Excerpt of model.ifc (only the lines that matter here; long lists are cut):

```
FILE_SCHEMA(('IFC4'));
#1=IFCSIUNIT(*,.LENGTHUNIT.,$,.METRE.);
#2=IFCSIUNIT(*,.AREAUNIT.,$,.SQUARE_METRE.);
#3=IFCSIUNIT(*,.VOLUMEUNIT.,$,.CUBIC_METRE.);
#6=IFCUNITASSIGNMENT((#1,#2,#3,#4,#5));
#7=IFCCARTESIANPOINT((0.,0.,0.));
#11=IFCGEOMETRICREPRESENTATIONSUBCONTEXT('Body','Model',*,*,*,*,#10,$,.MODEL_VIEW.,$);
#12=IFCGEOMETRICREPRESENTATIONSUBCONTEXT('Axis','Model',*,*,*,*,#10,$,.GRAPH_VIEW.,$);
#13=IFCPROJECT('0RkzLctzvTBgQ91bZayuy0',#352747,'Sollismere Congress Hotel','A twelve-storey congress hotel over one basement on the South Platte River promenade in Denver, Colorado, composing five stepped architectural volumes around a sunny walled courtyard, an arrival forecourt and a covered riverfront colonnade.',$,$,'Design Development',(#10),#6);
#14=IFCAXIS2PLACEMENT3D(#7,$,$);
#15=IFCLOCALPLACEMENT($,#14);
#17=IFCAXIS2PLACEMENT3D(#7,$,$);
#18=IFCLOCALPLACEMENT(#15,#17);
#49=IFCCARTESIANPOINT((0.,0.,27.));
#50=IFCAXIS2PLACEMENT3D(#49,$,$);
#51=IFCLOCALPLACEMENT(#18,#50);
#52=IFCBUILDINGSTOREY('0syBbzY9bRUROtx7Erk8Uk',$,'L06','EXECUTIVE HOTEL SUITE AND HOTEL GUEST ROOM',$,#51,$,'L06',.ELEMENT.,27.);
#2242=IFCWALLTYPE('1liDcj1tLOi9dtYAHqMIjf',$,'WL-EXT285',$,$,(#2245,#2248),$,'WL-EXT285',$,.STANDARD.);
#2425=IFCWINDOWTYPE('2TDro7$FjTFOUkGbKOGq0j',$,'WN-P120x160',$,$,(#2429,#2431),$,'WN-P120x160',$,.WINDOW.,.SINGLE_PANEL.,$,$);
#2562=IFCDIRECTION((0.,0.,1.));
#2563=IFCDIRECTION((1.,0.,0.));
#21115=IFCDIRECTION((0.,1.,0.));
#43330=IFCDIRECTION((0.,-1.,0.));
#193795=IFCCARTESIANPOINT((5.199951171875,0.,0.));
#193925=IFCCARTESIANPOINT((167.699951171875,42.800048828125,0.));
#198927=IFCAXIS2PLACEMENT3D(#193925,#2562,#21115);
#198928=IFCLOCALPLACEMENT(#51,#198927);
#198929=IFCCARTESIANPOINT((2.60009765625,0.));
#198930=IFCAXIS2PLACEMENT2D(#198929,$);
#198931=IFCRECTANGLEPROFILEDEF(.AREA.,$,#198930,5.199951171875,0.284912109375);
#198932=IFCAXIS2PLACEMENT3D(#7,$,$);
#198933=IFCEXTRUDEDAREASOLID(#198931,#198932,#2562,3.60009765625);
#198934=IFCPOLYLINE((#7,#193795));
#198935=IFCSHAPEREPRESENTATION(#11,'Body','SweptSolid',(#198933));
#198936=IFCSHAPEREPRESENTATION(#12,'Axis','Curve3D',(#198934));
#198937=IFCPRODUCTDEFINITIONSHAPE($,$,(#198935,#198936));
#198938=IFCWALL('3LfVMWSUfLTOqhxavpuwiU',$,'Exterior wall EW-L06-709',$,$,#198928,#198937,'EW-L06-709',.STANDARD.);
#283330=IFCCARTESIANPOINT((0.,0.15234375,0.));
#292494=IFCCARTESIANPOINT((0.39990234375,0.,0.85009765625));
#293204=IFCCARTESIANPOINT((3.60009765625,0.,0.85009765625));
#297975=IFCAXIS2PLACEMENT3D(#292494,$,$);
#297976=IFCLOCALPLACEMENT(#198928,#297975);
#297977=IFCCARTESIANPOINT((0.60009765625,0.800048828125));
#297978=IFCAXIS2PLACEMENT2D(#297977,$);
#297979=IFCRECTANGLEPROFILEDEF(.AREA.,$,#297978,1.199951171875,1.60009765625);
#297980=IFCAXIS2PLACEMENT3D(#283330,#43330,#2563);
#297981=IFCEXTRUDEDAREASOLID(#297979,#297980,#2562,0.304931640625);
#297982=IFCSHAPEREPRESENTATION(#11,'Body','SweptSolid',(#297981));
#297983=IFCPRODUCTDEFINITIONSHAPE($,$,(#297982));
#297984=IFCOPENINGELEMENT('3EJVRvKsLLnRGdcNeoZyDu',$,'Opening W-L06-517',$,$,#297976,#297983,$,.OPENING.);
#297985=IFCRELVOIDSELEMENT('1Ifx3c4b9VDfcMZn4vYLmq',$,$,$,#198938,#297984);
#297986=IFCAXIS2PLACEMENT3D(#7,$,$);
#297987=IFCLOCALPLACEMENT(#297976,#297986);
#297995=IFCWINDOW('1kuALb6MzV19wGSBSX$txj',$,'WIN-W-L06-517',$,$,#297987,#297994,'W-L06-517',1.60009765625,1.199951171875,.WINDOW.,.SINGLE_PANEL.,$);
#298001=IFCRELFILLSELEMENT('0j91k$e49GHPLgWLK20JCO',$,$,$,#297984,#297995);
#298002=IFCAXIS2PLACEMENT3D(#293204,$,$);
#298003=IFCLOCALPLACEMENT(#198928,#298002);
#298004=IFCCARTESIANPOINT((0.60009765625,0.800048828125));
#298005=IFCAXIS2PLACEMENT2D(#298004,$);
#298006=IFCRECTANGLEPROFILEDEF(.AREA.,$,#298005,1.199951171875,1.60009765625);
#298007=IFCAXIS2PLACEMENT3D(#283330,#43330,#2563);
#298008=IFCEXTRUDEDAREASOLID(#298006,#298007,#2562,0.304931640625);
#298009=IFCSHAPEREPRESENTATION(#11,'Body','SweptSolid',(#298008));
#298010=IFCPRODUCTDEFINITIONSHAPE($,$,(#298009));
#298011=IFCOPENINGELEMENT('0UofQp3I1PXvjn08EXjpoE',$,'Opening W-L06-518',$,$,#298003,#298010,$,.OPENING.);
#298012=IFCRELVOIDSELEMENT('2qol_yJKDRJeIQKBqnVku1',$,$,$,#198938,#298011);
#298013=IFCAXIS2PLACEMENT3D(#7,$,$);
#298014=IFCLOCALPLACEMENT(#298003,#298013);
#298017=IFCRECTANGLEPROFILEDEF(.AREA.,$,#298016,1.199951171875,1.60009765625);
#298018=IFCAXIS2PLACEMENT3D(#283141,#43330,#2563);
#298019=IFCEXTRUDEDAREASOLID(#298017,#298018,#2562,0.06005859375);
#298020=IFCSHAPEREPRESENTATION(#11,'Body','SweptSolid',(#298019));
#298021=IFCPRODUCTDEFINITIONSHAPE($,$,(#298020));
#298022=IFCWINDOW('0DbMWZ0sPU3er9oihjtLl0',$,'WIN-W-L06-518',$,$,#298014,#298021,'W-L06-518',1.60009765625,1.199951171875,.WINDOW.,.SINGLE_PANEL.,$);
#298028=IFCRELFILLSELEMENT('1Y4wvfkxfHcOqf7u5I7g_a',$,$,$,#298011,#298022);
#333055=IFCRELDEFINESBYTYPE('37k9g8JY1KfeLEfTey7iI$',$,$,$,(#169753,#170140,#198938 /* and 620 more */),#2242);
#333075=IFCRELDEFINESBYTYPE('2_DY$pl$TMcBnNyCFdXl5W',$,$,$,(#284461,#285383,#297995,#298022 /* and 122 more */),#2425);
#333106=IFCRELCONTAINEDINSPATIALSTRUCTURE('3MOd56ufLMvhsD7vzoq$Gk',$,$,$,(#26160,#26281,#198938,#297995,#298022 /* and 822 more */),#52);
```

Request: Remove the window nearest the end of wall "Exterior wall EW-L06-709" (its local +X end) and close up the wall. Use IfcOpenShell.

```python
import ifcopenshell
import ifcopenshell.api.feature
import ifcopenshell.api.root
import ifcopenshell.geom
import ifcopenshell.util.shape

model = ifcopenshell.open("model.ifc")
settings = ifcopenshell.geom.settings()


def volume(element):
    """Net volume in cubic metres, openings subtracted."""
    shape = ifcopenshell.geom.create_shape(settings, element)
    return ifcopenshell.util.shape.get_volume(shape.geometry)


window = model.by_id(298022)
opening = window.FillsVoids[0].RelatingOpeningElement
wall = opening.VoidsElements[0].RelatingBuildingElement
before = volume(wall)

ifcopenshell.api.root.remove_product(model, product=window)
ifcopenshell.api.feature.remove_feature(model, feature=opening)

after = volume(wall)

print(f"wall volume {before:.3f} -> {after:.3f} m3")

model.write("model_edited.ifc")
```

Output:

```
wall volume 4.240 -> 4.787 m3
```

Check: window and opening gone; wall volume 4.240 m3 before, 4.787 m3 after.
